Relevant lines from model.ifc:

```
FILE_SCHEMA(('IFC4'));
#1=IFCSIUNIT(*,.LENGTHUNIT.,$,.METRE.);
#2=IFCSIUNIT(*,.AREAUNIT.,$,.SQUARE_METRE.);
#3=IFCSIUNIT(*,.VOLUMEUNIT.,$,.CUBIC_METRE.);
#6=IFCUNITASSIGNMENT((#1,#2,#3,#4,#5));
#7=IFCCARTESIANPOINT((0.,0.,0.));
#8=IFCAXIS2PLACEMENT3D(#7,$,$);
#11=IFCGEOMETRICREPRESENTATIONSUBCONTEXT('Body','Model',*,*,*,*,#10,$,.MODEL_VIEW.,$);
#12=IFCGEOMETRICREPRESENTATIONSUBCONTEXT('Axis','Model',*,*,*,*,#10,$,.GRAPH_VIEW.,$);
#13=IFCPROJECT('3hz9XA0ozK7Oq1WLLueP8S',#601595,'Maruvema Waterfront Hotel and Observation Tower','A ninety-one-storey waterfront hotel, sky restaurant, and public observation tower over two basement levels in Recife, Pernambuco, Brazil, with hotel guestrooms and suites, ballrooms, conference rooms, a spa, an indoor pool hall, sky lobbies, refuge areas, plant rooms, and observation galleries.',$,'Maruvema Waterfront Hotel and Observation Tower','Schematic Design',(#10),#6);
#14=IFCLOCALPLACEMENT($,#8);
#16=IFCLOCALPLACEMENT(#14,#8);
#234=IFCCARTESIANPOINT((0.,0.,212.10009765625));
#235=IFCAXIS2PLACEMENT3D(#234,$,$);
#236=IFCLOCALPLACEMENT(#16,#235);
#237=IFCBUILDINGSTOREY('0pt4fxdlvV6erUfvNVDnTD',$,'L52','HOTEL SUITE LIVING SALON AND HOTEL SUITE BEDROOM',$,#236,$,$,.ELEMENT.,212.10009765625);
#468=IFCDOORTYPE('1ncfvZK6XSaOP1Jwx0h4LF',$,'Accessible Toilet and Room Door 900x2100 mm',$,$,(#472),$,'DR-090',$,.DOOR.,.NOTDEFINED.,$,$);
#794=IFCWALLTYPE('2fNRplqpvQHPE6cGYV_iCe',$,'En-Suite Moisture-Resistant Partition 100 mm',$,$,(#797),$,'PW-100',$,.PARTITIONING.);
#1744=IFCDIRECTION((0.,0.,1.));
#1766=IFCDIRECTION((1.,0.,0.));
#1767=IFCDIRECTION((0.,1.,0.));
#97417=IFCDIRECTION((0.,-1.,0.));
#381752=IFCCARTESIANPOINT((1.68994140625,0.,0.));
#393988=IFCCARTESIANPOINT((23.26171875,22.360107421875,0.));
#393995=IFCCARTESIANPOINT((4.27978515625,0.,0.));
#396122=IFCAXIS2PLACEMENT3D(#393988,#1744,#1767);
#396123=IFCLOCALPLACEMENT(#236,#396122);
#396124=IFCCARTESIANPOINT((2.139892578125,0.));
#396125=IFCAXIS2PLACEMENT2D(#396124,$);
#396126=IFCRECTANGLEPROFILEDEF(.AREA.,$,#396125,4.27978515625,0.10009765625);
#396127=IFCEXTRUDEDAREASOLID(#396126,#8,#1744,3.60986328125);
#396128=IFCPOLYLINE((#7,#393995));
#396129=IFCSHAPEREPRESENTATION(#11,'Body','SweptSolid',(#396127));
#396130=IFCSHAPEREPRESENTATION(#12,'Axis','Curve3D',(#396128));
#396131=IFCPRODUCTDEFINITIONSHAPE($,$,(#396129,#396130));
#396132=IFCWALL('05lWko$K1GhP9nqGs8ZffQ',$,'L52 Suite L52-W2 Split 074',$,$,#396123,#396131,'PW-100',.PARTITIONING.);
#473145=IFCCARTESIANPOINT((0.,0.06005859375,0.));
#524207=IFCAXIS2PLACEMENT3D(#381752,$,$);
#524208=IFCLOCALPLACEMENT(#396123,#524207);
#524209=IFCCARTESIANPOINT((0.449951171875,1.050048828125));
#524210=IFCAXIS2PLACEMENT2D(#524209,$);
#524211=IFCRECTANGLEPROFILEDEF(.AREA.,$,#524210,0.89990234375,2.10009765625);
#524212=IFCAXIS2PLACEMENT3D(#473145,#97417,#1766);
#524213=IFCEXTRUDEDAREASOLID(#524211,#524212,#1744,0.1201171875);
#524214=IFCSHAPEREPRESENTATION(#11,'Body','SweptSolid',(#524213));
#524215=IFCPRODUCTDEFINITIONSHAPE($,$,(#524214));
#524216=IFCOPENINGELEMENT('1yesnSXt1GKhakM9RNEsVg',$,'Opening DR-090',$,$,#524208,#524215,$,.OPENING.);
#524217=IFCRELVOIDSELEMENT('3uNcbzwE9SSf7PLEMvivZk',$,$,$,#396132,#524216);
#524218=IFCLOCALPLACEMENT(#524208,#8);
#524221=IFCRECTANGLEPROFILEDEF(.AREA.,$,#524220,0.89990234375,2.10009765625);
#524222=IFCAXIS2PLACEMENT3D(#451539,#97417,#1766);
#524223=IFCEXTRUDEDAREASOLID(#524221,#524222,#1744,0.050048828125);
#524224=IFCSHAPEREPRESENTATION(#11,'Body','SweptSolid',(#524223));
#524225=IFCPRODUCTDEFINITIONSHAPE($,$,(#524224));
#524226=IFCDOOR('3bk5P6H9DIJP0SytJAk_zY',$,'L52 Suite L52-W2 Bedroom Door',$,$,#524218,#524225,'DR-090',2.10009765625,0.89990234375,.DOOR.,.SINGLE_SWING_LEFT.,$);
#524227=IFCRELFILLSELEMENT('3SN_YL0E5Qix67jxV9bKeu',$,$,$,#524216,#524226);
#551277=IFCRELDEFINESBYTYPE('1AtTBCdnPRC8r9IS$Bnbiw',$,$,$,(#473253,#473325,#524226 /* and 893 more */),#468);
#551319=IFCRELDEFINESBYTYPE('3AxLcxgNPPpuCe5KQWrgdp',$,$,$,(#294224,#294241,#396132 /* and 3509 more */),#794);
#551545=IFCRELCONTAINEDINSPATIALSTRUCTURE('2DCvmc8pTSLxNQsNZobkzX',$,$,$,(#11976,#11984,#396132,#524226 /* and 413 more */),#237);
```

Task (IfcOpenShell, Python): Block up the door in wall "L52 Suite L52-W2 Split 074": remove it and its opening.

```python
import ifcopenshell
import ifcopenshell.api.feature
import ifcopenshell.api.root
import ifcopenshell.geom
import ifcopenshell.util.shape

model = ifcopenshell.open("model.ifc")
settings = ifcopenshell.geom.settings()


def volume(element):
    """Net volume in cubic metres, openings subtracted."""
    shape = ifcopenshell.geom.create_shape(settings, element)
    return ifcopenshell.util.shape.get_volume(shape.geometry)


door = model.by_guid("3bk5P6H9DIJP0SytJAk_zY")
opening = door.FillsVoids[0].RelatingOpeningElement
wall = opening.VoidsElements[0].RelatingBuildingElement
before = volume(wall)

ifcopenshell.api.root.remove_product(model, product=door)
ifcopenshell.api.feature.remove_feature(model, feature=opening)

after = volume(wall)

print(f"wall volume {before:.3f} -> {after:.3f} m3")

model.write("model-out.ifc")
```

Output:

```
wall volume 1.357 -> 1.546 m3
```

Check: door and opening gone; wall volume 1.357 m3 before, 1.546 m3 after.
